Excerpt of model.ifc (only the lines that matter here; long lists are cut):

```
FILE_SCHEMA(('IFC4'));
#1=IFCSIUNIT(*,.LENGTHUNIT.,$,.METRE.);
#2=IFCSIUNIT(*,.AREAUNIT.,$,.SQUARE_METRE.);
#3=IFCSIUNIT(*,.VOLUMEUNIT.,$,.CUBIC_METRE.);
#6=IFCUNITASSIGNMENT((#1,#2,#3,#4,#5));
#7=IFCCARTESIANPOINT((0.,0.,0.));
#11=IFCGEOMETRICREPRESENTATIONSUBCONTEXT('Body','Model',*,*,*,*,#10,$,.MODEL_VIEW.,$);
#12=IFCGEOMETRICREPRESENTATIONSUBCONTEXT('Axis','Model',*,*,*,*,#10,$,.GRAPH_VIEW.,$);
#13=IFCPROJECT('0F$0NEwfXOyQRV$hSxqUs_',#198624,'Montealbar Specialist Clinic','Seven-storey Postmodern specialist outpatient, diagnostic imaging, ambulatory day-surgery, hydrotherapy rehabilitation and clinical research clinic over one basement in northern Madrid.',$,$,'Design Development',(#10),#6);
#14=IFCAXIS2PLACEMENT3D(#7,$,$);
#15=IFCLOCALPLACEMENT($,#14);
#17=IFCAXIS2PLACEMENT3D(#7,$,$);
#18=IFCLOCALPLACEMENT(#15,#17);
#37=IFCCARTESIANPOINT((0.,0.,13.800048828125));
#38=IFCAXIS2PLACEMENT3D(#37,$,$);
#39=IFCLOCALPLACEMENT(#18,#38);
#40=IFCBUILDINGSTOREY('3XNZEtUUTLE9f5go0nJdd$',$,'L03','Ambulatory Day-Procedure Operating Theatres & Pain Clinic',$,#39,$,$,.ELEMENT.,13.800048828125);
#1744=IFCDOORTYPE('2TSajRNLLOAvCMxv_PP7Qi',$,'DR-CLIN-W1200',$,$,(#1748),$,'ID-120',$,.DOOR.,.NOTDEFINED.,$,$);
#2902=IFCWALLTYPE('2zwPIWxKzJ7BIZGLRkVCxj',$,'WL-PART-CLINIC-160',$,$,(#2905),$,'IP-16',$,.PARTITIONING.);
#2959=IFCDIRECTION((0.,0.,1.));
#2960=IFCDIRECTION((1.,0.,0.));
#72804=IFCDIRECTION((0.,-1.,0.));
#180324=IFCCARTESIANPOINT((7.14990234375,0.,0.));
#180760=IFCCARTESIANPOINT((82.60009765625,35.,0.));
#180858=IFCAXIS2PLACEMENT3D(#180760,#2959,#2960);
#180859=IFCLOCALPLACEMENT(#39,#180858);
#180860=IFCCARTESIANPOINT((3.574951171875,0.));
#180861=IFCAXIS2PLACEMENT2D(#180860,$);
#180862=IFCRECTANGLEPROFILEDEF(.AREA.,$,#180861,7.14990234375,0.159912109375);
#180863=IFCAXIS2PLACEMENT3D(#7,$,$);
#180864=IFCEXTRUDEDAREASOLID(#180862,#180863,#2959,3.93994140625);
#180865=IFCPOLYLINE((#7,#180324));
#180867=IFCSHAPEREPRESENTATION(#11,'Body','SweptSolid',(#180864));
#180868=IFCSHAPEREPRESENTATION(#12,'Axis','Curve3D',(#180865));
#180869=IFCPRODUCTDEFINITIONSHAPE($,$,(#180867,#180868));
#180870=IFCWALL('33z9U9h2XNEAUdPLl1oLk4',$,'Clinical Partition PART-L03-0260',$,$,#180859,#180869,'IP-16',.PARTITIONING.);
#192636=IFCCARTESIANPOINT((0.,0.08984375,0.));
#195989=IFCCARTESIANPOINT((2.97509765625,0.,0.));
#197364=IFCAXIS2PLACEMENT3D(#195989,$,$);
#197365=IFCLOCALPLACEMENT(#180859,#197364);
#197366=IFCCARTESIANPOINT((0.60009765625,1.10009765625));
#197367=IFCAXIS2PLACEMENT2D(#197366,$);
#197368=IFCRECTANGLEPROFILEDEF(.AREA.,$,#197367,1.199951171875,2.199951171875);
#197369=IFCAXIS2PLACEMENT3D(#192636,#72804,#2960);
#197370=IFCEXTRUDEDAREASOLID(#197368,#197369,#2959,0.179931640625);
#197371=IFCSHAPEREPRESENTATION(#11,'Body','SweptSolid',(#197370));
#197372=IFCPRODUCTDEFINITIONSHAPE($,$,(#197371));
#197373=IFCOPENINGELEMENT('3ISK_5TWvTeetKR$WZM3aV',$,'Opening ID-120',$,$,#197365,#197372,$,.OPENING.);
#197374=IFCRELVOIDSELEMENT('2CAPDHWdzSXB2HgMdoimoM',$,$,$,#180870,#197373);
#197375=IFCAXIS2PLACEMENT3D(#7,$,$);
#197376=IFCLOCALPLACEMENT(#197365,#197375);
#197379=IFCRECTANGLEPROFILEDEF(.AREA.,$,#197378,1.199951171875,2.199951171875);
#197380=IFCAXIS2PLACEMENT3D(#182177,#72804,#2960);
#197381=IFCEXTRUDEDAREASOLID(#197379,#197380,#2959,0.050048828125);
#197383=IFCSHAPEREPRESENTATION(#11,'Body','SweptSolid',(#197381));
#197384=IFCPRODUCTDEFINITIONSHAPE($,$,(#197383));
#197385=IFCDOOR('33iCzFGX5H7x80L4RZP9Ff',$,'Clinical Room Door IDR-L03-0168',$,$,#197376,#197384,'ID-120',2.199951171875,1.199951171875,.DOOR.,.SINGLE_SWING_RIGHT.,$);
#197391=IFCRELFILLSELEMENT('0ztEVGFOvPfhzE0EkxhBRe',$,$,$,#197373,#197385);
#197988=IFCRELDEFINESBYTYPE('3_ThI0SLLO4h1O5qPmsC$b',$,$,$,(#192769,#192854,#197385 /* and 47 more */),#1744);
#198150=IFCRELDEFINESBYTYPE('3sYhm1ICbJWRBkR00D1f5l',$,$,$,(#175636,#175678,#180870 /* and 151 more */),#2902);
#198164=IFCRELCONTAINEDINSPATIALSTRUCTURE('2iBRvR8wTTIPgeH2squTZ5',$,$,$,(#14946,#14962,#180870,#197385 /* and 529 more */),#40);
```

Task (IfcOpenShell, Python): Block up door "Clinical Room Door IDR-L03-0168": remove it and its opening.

```python
import ifcopenshell
import ifcopenshell.api.feature
import ifcopenshell.api.root
import ifcopenshell.geom
import ifcopenshell.util.shape

model = ifcopenshell.open("model.ifc")
settings = ifcopenshell.geom.settings()


def volume(element):
    """Net volume in cubic metres, openings subtracted."""
    shape = ifcopenshell.geom.create_shape(settings, element)
    return ifcopenshell.util.shape.get_volume(shape.geometry)


door = model.by_guid("33iCzFGX5H7x80L4RZP9Ff")
opening = door.FillsVoids[0].RelatingOpeningElement
wall = opening.VoidsElements[0].RelatingBuildingElement
before = volume(wall)

ifcopenshell.api.root.remove_product(model, product=door)
ifcopenshell.api.feature.remove_feature(model, feature=opening)

after = volume(wall)

print(f"wall volume {before:.3f} -> {after:.3f} m3")

model.write("model-out.ifc")
```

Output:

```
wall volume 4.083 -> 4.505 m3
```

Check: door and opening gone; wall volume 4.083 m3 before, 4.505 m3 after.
